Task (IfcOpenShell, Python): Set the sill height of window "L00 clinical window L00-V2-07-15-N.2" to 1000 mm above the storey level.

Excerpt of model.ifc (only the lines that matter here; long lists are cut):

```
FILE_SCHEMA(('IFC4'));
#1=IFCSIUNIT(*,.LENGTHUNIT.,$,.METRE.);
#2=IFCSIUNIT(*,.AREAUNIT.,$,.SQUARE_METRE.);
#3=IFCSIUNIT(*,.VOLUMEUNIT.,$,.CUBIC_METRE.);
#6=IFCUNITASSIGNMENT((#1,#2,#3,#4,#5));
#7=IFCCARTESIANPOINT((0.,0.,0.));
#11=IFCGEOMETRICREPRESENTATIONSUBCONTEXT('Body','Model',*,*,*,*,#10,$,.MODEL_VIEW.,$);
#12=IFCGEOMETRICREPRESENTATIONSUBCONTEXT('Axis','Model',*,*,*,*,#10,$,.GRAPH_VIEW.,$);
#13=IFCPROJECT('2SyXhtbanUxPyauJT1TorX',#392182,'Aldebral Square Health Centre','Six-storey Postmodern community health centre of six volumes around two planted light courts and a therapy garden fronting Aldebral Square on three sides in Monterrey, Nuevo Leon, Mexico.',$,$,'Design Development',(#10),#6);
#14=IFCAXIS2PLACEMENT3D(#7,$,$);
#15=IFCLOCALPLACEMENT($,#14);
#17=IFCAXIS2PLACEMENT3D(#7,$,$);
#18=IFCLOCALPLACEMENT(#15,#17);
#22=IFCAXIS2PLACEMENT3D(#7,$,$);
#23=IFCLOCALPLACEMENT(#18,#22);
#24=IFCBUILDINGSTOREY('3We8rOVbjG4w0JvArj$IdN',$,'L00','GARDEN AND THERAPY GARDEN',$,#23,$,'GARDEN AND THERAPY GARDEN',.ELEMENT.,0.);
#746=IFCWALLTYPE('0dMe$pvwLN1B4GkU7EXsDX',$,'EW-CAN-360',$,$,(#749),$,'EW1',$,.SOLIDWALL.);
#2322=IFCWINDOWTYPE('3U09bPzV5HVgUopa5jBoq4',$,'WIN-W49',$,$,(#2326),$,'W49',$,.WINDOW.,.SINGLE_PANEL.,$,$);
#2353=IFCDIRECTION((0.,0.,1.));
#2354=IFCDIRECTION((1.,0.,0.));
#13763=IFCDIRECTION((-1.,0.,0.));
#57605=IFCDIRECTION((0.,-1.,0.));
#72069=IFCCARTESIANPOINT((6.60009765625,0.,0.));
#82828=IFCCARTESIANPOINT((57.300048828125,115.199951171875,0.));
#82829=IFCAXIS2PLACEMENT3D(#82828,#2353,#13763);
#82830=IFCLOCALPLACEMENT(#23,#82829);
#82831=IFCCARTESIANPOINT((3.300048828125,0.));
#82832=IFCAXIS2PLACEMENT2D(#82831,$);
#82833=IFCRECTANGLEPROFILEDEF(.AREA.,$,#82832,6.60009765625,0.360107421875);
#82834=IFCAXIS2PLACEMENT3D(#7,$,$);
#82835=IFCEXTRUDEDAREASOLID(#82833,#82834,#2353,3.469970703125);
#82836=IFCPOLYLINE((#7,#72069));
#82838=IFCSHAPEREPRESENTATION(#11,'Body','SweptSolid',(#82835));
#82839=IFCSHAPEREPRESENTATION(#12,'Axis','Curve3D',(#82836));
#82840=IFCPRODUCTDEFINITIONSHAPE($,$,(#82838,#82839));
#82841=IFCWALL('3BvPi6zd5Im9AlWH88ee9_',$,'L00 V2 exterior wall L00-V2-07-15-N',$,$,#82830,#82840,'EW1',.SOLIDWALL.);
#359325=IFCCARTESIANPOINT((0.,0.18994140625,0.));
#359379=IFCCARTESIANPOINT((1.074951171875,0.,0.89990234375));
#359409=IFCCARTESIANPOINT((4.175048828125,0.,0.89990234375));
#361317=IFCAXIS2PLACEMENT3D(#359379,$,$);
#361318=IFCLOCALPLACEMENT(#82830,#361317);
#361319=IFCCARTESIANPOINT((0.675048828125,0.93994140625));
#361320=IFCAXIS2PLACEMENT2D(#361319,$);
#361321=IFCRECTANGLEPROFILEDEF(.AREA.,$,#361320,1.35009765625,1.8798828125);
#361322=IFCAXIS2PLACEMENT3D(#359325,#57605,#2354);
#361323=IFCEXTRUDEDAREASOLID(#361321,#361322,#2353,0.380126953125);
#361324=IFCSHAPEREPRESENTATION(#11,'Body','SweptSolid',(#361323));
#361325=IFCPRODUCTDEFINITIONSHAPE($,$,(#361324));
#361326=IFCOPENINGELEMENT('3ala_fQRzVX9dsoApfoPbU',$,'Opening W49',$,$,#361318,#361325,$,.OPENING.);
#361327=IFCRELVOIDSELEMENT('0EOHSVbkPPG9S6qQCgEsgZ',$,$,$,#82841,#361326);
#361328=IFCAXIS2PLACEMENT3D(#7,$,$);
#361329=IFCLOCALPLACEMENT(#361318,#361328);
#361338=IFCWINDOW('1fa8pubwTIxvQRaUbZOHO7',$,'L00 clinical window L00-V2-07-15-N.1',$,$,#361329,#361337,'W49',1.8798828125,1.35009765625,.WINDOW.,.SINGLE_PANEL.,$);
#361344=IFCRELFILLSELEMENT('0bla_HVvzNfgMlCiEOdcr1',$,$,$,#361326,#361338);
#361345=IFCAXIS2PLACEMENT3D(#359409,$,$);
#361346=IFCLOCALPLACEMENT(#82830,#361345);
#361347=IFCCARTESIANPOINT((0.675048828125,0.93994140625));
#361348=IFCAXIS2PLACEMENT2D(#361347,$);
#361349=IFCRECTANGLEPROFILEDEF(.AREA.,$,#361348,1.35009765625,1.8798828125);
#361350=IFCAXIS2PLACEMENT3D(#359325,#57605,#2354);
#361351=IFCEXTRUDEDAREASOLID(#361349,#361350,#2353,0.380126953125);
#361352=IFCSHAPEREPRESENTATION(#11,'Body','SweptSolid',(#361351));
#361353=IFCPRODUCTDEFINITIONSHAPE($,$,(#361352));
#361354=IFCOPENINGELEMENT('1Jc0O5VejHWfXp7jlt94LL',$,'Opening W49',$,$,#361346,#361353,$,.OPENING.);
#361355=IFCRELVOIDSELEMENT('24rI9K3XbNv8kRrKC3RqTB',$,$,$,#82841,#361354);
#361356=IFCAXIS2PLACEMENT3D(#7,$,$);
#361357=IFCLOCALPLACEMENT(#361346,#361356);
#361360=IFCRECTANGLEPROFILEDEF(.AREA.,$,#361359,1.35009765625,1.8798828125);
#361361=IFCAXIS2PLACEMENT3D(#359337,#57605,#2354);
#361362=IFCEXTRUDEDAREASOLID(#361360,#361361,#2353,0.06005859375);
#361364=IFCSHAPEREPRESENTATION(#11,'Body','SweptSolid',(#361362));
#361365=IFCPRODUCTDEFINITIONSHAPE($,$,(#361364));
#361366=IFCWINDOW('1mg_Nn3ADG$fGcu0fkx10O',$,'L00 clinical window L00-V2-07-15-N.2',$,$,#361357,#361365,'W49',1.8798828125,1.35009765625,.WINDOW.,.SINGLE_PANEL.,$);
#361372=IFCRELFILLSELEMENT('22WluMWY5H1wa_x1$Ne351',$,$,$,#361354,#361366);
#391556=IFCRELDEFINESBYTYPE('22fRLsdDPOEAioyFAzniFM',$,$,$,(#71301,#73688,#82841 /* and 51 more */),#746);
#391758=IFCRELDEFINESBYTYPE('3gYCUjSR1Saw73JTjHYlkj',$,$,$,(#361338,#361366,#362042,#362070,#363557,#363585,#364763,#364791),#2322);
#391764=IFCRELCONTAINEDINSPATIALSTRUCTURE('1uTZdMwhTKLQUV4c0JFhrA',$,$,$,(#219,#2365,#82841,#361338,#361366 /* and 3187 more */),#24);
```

```python
import numpy as np
import ifcopenshell
import ifcopenshell.api.geometry
import ifcopenshell.geom
import ifcopenshell.util.element
import ifcopenshell.util.placement
import ifcopenshell.util.shape
import ifcopenshell.util.unit

model = ifcopenshell.open("model.ifc")
unit_scale = ifcopenshell.util.unit.calculate_unit_scale(model)

window = model.by_guid("1mg_Nn3ADG$fGcu0fkx10O")
opening = window.FillsVoids[0].RelatingOpeningElement
storey = ifcopenshell.util.element.get_container(window, ifc_class="IfcBuildingStorey")
level = ifcopenshell.util.placement.get_local_placement(storey.ObjectPlacement)[2, 3]

# The opening's origin need not be at the sill, so measure its lowest point.
shape = ifcopenshell.geom.create_shape(ifcopenshell.geom.settings(), opening)
bottom = ifcopenshell.util.shape.get_shape_bottom_elevation(shape, shape.geometry) / unit_scale
dz = level + 1 / unit_scale - bottom

shift = np.array([0.0, 0.0, dz])
# The window is placed relative to its opening, so it follows when the opening moves.
matrix = ifcopenshell.util.placement.get_local_placement(opening.ObjectPlacement)
matrix[:3, 3] += shift
ifcopenshell.api.geometry.edit_object_placement(
    model, product=opening, matrix=matrix, is_si=False, should_transform_children=True
)

print(f"moved by {dz * unit_scale:+.3f} m")

model.write("model_v2.ifc")
```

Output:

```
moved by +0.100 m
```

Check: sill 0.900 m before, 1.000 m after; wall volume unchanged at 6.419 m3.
